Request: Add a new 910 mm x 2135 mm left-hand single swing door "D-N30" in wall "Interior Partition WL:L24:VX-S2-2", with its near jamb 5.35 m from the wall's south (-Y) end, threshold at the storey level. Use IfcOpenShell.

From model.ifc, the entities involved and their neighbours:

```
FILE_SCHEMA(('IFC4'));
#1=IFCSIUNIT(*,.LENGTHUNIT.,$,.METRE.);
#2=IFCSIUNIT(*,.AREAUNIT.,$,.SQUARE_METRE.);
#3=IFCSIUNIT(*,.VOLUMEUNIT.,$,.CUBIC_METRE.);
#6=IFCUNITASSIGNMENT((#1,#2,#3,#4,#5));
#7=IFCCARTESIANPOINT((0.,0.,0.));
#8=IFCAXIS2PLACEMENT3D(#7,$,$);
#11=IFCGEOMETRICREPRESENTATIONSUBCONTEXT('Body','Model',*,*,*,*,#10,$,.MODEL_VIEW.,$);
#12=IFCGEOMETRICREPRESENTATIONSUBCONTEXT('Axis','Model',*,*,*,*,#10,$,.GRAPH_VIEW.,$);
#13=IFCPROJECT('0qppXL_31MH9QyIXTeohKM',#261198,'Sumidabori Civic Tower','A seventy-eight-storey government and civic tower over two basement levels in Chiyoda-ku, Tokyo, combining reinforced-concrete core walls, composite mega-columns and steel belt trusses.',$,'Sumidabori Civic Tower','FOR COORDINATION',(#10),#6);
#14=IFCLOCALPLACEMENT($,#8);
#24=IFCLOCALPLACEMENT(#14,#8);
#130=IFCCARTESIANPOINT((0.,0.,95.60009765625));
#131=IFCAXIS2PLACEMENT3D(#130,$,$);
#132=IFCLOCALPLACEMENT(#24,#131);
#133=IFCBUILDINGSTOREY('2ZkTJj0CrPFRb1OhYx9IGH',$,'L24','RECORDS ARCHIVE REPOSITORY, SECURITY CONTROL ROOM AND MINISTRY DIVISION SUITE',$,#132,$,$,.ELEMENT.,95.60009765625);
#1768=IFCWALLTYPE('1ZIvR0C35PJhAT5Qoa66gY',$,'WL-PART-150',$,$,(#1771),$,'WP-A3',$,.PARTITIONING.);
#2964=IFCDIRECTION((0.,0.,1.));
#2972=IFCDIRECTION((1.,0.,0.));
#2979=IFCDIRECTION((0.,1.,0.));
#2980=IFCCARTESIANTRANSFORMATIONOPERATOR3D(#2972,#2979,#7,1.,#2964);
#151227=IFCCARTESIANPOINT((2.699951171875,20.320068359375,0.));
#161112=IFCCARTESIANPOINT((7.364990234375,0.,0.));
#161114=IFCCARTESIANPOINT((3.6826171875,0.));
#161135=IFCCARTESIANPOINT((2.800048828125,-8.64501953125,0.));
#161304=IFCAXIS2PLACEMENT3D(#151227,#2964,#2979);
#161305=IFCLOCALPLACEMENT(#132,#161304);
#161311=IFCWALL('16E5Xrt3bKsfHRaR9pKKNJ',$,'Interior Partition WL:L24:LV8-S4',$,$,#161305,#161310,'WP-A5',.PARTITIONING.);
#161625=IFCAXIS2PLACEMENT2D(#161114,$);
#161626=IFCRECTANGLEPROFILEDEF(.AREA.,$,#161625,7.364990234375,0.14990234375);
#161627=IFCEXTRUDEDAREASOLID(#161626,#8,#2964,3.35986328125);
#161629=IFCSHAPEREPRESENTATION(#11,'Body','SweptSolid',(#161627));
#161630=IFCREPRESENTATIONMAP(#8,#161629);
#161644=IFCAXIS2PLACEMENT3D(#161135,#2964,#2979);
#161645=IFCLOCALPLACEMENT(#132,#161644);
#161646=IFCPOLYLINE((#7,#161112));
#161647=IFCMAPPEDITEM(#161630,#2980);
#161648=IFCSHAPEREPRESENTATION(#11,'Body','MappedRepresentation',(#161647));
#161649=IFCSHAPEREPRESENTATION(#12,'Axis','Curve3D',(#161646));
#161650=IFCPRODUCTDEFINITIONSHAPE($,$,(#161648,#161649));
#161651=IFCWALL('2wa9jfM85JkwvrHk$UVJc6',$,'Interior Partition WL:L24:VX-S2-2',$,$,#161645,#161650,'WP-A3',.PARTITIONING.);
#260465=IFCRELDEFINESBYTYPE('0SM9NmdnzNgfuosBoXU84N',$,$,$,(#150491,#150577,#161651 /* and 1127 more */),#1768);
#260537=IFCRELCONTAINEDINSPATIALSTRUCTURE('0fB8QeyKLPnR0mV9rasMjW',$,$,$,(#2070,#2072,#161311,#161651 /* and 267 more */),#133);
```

```python
import numpy as np
import ifcopenshell
import ifcopenshell.api.feature
import ifcopenshell.api.geometry
import ifcopenshell.api.root
import ifcopenshell.api.spatial
import ifcopenshell.geom
import ifcopenshell.util.element
import ifcopenshell.util.placement
import ifcopenshell.util.representation
import ifcopenshell.util.shape
import ifcopenshell.util.unit

model = ifcopenshell.open("model.ifc")
unit_scale = ifcopenshell.util.unit.calculate_unit_scale(model)
settings = ifcopenshell.geom.settings()


def volume(element):
    """Net volume in cubic metres, openings subtracted."""
    shape = ifcopenshell.geom.create_shape(settings, element)
    return ifcopenshell.util.shape.get_volume(shape.geometry)


wall = model.by_guid("2wa9jfM85JkwvrHk$UVJc6")
storey = ifcopenshell.util.element.get_container(wall, ifc_class="IfcBuildingStorey")
context = ifcopenshell.util.representation.get_context(model, "Model", "Body", "MODEL_VIEW")
before = volume(wall)

width, height, from_end, sill = 0.91, 2.135, 5.35, 0.0  # metres

# The wall runs along its own X axis, and the end named is its -X end.
wall_shape = ifcopenshell.geom.create_shape(settings, wall)
x, y, z = ifcopenshell.util.shape.get_vertices(wall_shape.geometry).T
start = x.min() + from_end
face, thickness = float(y.min()), float(y.max() - y.min())
wall_matrix = ifcopenshell.util.placement.get_local_placement(wall.ObjectPlacement)
level = ifcopenshell.util.placement.get_local_placement(storey.ObjectPlacement)[2, 3]


def in_wall(x, y):
    """Placement at x, y metres in the wall's axes, at sill height."""
    matrix = wall_matrix.copy()
    matrix[:, 3] = wall_matrix @ np.array([x / unit_scale, y / unit_scale, 0.0, 1.0])
    matrix[2, 3] = level + sill / unit_scale
    return matrix


# Opening: a box that overshoots both wall faces by 50 mm.
opening = ifcopenshell.api.root.create_entity(model, ifc_class="IfcOpeningElement", predefined_type="OPENING")
box = ifcopenshell.api.geometry.add_wall_representation(
    model, context=context, length=width, height=height, thickness=thickness + 0.1
)
ifcopenshell.api.geometry.assign_representation(model, product=opening, representation=box)
ifcopenshell.api.geometry.edit_object_placement(model, product=opening, matrix=in_wall(start, face - 0.05), is_si=False)
ifcopenshell.api.feature.add_feature(model, feature=opening, element=wall)

door = ifcopenshell.api.root.create_entity(model, ifc_class="IfcDoor", name="D-N30", predefined_type="DOOR")
door.OverallWidth, door.OverallHeight = width / unit_scale, height / unit_scale
door.OperationType = "SINGLE_SWING_LEFT"
body = ifcopenshell.api.geometry.add_door_representation(
    model,
    context=context,
    overall_width=door.OverallWidth,
    overall_height=door.OverallHeight,
    operation_type="SINGLE_SWING_LEFT",
    lining_properties={"LiningDepth": thickness / unit_scale, "ThresholdDepth": thickness / unit_scale},
)
ifcopenshell.api.geometry.assign_representation(model, product=door, representation=body)
ifcopenshell.api.spatial.assign_container(model, products=[door], relating_structure=storey)
ifcopenshell.api.feature.add_filling(model, opening=opening, element=door)

# The lining spans the wall, so the door starts at the wall face.
ifcopenshell.api.geometry.edit_object_placement(model, product=door, matrix=in_wall(start, face), is_si=False)

after = volume(wall)

print(f"wall volume {before:.3f} -> {after:.3f} m3")

model.write("model_rev.ifc")
```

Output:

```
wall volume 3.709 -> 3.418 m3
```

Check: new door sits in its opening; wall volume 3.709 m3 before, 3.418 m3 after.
